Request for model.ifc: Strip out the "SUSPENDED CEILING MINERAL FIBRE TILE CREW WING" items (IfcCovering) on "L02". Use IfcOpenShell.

First a look at what the model holds.

```python
import ifcopenshell
import ifcopenshell.util.element

model = ifcopenshell.open("model.ifc")
print(model.schema)
storey = next(s for s in model.by_type("IfcBuildingStorey") if s.Name == "L02")
coverings = [e for e in ifcopenshell.util.element.get_decomposition(storey) if e.is_a("IfcCovering")]
seen = {}
for e in coverings:
    element_type = ifcopenshell.util.element.get_type(e)
    name = element_type.Name if element_type not in (None, e) else None
    seen[name] = seen.get(name, 0) + 1
for name, count in sorted(seen.items(), key=str):
    print(count, "x", name)
```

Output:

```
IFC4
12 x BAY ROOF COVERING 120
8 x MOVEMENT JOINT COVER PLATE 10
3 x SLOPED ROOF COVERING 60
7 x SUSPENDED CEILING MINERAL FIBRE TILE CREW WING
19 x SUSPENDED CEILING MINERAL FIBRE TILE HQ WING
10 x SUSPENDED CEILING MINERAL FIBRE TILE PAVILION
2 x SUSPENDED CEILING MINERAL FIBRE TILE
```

```python
import ifcopenshell
import ifcopenshell.api.root
import ifcopenshell.util.element

model = ifcopenshell.open("model.ifc")

storey = next(s for s in model.by_type("IfcBuildingStorey") if s.Name == "L02")
coverings = [e for e in ifcopenshell.util.element.get_decomposition(storey) if e.is_a("IfcCovering")]
targets = [e for e in coverings if (t := ifcopenshell.util.element.get_type(e)) not in (None, e) and t.Name == "SUSPENDED CEILING MINERAL FIBRE TILE CREW WING"]

for e in targets:
    ifcopenshell.api.root.remove_product(model, product=e)
print(len(targets), "removed")

model.write("model-out.ifc")
```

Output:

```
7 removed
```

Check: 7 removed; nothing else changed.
